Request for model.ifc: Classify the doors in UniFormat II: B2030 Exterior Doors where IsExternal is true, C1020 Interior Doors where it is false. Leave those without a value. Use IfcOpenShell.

First a look at what the model holds.

```python
import ifcopenshell
import ifcopenshell.util.element

model = ifcopenshell.open("model.ifc")
print(model.schema)
print("classifications:", [c.Name for c in model.by_type("IfcClassification")])
values = [ifcopenshell.util.element.get_pset(e, "Pset_DoorCommon", "IsExternal") for e in model.by_type("IfcDoor")]
for value in (True, False, None):
    print("IsExternal", value, values.count(value))
```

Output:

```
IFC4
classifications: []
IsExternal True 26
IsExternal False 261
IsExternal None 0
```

```python
import ifcopenshell
import ifcopenshell.api.classification
import ifcopenshell.util.element

model = ifcopenshell.open("model.ifc")

system = ifcopenshell.api.classification.add_classification(model, classification="UniFormat II")

doors = model.by_type("IfcDoor")
external = {e: ifcopenshell.util.element.get_pset(e, "Pset_DoorCommon", "IsExternal") for e in doors}
for flag, code, name in ((True, "B2030", "Exterior Doors"), (False, "C1020", "Interior Doors")):
    products = [e for e in doors if external[e] is flag]
    ifcopenshell.api.classification.add_reference(
        model, products=products, classification=system, identification=code, name=name
    )
    print(code, len(products))

model.write("model-out.ifc")
```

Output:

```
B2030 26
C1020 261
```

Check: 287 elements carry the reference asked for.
